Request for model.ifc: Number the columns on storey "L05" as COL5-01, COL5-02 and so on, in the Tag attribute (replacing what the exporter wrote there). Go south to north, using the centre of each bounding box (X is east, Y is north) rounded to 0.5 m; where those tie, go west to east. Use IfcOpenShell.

First a look at what the model holds.

```python
import ifcopenshell
import ifcopenshell.util.element
import ifcopenshell.util.placement

model = ifcopenshell.open("model.ifc")
print(model.schema)
storey = next(s for s in model.by_type("IfcBuildingStorey") if s.Name == "L05")
columns = [e for e in ifcopenshell.util.element.get_decomposition(storey) if e.is_a("IfcColumn")]
for e in sorted(columns, key=lambda e: e.id()):
    origin = ifcopenshell.util.placement.get_local_placement(e.ObjectPlacement)[:3, 3]
    print(e.id(), e.Tag, e.Name, origin.round(2) + 0.0, sep=" | ")
```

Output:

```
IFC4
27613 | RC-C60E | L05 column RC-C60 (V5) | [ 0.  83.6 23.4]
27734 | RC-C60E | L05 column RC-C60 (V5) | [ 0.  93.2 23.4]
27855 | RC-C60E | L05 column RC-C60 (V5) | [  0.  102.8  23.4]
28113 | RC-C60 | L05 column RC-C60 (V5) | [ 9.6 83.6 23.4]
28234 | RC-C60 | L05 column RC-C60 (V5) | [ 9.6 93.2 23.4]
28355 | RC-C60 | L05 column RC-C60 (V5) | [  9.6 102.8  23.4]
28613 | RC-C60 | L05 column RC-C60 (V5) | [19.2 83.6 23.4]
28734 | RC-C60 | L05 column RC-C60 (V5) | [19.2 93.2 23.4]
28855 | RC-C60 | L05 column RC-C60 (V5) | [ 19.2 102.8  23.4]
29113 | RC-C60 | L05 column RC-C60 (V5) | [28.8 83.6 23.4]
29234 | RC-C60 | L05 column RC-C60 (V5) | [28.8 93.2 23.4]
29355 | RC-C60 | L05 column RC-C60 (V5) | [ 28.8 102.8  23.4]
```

```python
import ifcopenshell
import ifcopenshell.geom
import ifcopenshell.util.element
import ifcopenshell.util.shape

model = ifcopenshell.open("model.ifc")
settings = ifcopenshell.geom.settings()
settings.set("use-world-coords", True)


def centre(element):
    shape = ifcopenshell.geom.create_shape(settings, element)
    return ifcopenshell.util.shape.get_bbox_centroid(shape.geometry)


storey = next(s for s in model.by_type("IfcBuildingStorey") if s.Name == "L05")
columns = [e for e in ifcopenshell.util.element.get_decomposition(storey) if e.is_a("IfcColumn")]

# Insertion points can sit at a corner or the storey origin, so sort by the geometry (in metres).
centres = {e: centre(e) for e in columns}
columns.sort(key=lambda e: (round(centres[e][1] / 0.5), centres[e][0]))

for i, e in enumerate(columns, start=1):
    number = f"COL5-{i:02d}"
    e.Tag = number
    print(e.id(), number)

model.write("model_edited.ifc")
```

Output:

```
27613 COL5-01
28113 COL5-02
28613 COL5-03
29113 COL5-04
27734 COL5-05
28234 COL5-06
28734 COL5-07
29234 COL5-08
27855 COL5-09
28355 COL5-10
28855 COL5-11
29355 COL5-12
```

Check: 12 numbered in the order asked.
